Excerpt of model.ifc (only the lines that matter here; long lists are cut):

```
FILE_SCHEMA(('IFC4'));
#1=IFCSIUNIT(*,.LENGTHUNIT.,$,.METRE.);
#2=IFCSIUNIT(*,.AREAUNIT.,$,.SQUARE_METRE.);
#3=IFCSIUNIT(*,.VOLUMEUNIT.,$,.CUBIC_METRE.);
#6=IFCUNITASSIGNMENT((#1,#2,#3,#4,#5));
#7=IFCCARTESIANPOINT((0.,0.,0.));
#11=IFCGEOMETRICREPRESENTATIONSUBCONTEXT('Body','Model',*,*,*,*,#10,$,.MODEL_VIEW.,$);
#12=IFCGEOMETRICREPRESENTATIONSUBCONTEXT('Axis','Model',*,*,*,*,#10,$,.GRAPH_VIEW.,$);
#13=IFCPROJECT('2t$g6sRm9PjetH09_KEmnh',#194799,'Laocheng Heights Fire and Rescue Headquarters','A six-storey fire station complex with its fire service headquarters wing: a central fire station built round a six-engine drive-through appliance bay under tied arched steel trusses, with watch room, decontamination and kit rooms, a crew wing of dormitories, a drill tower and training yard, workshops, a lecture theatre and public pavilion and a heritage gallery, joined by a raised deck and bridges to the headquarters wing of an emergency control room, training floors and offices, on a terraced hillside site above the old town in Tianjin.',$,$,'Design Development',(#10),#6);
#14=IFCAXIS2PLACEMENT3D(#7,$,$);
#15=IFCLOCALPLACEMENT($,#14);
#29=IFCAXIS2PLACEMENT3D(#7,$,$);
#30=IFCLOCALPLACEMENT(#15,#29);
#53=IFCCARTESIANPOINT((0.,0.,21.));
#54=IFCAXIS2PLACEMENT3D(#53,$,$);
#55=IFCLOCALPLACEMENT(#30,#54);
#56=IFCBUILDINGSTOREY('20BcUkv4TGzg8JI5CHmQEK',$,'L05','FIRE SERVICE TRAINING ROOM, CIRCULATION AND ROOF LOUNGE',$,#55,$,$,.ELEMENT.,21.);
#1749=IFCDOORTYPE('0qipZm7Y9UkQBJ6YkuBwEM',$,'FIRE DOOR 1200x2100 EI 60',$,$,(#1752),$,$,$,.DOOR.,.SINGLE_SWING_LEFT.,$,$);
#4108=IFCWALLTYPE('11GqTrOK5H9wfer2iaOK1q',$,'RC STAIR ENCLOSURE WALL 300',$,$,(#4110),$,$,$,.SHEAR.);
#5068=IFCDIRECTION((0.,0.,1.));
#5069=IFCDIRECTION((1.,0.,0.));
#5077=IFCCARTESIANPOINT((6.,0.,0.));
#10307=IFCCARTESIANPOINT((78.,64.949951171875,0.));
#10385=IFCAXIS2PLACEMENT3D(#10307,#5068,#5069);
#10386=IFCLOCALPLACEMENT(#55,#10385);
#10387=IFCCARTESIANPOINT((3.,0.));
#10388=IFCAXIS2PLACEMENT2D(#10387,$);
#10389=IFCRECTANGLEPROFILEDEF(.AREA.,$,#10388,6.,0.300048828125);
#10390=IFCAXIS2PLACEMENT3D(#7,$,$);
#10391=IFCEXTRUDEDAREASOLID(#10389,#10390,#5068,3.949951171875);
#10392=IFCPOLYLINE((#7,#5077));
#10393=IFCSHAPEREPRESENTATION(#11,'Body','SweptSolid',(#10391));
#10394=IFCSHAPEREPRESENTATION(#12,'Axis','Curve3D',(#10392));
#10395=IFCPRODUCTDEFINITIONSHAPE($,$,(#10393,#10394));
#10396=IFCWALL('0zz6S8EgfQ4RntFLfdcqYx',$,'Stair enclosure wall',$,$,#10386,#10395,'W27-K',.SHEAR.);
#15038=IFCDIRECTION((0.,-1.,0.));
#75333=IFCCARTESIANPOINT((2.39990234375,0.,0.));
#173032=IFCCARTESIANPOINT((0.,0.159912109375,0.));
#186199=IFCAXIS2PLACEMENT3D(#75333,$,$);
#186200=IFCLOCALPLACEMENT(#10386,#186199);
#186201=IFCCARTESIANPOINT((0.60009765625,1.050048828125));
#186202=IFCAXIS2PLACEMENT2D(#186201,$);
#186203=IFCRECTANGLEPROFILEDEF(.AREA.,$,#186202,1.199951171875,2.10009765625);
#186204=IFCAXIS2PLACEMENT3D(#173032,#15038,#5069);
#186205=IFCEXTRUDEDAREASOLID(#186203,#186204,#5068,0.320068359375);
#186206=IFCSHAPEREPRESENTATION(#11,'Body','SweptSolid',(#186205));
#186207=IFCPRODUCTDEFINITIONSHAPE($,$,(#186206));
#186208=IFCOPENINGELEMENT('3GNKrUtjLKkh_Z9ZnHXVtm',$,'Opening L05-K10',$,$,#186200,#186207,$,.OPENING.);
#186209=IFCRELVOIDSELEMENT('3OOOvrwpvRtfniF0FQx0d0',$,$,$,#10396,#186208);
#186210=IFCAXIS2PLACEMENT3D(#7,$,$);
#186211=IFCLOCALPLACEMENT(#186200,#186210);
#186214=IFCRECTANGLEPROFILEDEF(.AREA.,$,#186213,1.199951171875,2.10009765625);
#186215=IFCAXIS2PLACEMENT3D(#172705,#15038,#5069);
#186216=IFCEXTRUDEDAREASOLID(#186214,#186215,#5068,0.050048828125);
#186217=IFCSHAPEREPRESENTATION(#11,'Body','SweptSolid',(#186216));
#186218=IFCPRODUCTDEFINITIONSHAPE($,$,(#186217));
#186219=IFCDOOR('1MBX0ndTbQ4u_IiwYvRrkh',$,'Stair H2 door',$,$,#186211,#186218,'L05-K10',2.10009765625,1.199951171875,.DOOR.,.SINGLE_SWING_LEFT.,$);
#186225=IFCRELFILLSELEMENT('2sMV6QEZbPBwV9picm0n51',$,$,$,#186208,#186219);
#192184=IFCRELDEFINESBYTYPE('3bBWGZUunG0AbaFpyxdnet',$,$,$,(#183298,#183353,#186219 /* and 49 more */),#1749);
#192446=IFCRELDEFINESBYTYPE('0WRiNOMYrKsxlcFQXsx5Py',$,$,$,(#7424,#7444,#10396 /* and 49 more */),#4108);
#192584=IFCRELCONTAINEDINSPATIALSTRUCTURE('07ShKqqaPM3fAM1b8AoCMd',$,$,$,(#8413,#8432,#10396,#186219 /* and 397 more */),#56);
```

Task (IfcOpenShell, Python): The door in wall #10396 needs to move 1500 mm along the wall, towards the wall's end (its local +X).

```python
import ifcopenshell
import ifcopenshell.api.geometry
import ifcopenshell.util.placement

model = ifcopenshell.open("model.ifc")

door = model.by_guid("1MBX0ndTbQ4u_IiwYvRrkh")
opening = door.FillsVoids[0].RelatingOpeningElement
wall = opening.VoidsElements[0].RelatingBuildingElement

wall_matrix = ifcopenshell.util.placement.get_local_placement(wall.ObjectPlacement)
shift = wall_matrix[:3, 0] * 1.5
before = ifcopenshell.util.placement.get_local_placement(door.ObjectPlacement)[:3, 3].copy()

# The door is placed relative to its opening, so it follows when the opening moves.
matrix = ifcopenshell.util.placement.get_local_placement(opening.ObjectPlacement)
matrix[:3, 3] += shift
ifcopenshell.api.geometry.edit_object_placement(
    model, product=opening, matrix=matrix, is_si=False, should_transform_children=True
)

after = ifcopenshell.util.placement.get_local_placement(door.ObjectPlacement)[:3, 3]
print("door moved by", (after - before).round(3) + 0.0)

model.write("model_rev.ifc")
```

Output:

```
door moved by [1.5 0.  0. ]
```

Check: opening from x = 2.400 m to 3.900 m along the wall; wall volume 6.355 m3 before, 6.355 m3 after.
